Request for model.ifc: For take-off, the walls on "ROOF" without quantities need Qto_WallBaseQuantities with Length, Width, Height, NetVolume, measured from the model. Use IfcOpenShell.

First a look at what the model holds.

```python
import ifcopenshell
import ifcopenshell.util.element
import ifcopenshell.util.unit

model = ifcopenshell.open("model.ifc")
print(model.schema)
for unit_type in ("LENGTHUNIT", "AREAUNIT", "VOLUMEUNIT"):
    print(unit_type, ifcopenshell.util.unit.calculate_unit_scale(model, unit_type))
storey = next(s for s in model.by_type("IfcBuildingStorey") if s.Name == "ROOF")
walls = [e for e in ifcopenshell.util.element.get_decomposition(storey) if e.is_a("IfcWall")]
for e in sorted(walls, key=lambda e: e.id()):
    print(e.id(), e.is_a(), e.Name, list(ifcopenshell.util.element.get_psets(e, qtos_only=True)), sep=" | ")
```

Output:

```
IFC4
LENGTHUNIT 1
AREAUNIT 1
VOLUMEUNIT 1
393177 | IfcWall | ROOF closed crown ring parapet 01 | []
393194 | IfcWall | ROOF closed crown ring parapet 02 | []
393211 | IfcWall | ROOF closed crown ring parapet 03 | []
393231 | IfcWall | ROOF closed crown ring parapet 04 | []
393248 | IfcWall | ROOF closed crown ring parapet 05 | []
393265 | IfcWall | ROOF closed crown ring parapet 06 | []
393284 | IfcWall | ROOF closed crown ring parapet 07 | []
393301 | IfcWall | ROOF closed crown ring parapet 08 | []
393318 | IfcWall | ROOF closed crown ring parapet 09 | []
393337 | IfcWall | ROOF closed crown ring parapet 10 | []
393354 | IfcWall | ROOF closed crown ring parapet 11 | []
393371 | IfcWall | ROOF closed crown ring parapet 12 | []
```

```python
import ifcopenshell
import ifcopenshell.api.pset
import ifcopenshell.geom
import ifcopenshell.util.element
import ifcopenshell.util.shape
import ifcopenshell.util.unit

model = ifcopenshell.open("model.ifc")
unit_scale = ifcopenshell.util.unit.calculate_unit_scale(model)
volume_scale = ifcopenshell.util.unit.calculate_unit_scale(model, "VOLUMEUNIT")
settings = ifcopenshell.geom.settings()

storey = next(s for s in model.by_type("IfcBuildingStorey") if s.Name == "ROOF")
walls = [e for e in ifcopenshell.util.element.get_decomposition(storey) if e.is_a("IfcWall")]

for e in sorted(walls, key=lambda e: e.id()):
    if ifcopenshell.util.element.get_psets(e, qtos_only=True, should_inherit=False):
        continue
    # Geometry comes back in metres, in the element's own axes.
    shape = ifcopenshell.geom.create_shape(settings, e)
    values = {
        "Length": ifcopenshell.util.shape.get_x(shape.geometry) / unit_scale,
        "Width": ifcopenshell.util.shape.get_y(shape.geometry) / unit_scale,
        "Height": ifcopenshell.util.shape.get_z(shape.geometry) / unit_scale,
        "NetVolume": ifcopenshell.util.shape.get_volume(shape.geometry) / volume_scale,
    }
    qto = ifcopenshell.api.pset.add_qto(model, product=e, name="Qto_WallBaseQuantities")
    ifcopenshell.api.pset.edit_qto(model, qto=qto, properties=values)
    print(e.id(), {k: round(v, 3) for k, v in values.items()})

model.write("model_rev.ifc")
```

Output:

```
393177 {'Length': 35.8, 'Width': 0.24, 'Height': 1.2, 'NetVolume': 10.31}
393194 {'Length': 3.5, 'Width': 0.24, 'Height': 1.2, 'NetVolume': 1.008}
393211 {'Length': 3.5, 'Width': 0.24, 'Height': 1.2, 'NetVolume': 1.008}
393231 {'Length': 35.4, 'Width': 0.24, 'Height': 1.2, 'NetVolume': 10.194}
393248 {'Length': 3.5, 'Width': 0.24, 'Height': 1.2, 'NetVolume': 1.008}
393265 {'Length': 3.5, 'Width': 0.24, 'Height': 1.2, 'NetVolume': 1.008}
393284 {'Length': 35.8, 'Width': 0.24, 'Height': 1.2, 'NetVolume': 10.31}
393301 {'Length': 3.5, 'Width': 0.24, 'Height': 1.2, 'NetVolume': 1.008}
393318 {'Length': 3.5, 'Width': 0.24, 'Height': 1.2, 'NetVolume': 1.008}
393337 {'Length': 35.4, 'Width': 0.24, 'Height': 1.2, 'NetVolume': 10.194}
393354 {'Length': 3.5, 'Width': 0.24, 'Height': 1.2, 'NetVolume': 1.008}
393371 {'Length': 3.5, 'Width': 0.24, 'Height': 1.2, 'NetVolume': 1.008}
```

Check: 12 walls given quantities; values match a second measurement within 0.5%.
